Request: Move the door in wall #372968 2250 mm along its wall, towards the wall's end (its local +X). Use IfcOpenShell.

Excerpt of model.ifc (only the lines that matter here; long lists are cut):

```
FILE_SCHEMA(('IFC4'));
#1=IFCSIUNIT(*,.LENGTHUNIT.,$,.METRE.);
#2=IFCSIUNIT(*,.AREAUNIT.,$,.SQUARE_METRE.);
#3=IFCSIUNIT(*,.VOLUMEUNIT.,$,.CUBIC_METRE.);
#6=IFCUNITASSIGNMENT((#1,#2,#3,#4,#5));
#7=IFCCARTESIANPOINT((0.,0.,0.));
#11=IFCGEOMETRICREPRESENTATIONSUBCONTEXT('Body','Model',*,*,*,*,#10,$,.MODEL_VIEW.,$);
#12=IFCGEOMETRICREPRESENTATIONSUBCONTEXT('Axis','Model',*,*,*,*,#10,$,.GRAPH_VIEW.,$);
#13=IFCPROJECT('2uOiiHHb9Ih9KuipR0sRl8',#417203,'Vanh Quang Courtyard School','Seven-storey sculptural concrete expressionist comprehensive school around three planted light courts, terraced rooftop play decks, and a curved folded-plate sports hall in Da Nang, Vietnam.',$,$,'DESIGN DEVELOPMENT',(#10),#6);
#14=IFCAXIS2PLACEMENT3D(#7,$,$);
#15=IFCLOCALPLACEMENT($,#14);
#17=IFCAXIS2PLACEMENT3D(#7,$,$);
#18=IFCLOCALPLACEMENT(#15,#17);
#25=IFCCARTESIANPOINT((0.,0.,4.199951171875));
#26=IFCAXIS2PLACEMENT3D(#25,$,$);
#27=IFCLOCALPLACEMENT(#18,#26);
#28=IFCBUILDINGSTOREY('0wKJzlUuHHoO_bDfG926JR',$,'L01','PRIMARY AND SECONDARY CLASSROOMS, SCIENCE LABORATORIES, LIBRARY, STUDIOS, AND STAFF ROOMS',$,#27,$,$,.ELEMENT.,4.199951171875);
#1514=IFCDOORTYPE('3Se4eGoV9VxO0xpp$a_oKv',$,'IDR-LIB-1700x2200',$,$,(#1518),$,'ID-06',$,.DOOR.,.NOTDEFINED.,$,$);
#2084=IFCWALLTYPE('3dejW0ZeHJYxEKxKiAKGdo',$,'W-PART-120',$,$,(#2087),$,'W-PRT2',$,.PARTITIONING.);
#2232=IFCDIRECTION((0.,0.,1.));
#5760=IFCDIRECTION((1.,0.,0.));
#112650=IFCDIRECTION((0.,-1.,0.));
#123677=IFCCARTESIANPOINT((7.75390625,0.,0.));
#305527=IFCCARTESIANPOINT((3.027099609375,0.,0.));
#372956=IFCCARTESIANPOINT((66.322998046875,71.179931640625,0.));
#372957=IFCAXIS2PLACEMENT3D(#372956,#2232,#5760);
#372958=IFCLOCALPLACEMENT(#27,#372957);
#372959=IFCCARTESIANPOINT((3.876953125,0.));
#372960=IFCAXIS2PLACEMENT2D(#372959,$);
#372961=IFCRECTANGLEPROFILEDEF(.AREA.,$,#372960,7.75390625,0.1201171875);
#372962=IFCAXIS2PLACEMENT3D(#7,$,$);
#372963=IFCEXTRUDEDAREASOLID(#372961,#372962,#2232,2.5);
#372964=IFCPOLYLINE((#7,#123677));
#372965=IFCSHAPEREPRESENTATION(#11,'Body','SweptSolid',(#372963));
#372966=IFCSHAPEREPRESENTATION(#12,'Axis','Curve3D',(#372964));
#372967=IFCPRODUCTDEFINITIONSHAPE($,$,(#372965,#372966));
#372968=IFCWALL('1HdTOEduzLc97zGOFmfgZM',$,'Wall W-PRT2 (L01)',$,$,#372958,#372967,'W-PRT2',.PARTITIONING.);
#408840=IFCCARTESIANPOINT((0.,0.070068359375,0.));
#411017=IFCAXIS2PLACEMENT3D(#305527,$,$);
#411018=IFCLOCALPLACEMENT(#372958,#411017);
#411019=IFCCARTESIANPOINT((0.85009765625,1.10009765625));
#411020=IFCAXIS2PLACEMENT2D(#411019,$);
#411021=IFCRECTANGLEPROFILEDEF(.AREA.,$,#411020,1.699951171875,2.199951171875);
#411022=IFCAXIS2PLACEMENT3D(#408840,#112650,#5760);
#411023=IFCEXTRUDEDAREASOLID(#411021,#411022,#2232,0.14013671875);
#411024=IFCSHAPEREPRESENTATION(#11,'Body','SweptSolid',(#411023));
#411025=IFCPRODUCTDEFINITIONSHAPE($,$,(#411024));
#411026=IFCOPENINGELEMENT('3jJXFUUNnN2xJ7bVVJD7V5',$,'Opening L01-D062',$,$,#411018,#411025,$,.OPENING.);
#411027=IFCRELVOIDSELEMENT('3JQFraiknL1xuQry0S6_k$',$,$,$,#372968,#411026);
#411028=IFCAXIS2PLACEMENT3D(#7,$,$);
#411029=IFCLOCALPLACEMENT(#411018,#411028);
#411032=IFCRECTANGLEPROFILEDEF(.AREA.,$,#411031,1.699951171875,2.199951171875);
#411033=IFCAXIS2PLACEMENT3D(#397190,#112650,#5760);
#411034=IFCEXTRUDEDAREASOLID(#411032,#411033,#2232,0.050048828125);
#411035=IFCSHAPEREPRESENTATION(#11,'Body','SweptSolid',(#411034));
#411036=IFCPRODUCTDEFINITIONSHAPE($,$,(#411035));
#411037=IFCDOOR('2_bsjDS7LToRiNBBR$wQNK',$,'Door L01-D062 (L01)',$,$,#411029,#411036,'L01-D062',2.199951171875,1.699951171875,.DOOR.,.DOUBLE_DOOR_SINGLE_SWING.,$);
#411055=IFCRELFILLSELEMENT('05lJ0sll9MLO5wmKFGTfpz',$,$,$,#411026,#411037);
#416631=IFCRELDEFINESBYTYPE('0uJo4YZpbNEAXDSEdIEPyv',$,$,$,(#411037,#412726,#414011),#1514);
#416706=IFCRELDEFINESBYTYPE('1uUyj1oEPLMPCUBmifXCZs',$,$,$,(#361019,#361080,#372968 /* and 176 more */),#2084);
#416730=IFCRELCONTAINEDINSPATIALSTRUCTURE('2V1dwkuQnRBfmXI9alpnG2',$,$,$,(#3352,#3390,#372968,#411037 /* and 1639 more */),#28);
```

```python
import ifcopenshell
import ifcopenshell.api.geometry
import ifcopenshell.util.placement

model = ifcopenshell.open("model.ifc")

door = model.by_guid("2_bsjDS7LToRiNBBR$wQNK")
opening = door.FillsVoids[0].RelatingOpeningElement
wall = opening.VoidsElements[0].RelatingBuildingElement

wall_matrix = ifcopenshell.util.placement.get_local_placement(wall.ObjectPlacement)
shift = wall_matrix[:3, 0] * 2.25
before = ifcopenshell.util.placement.get_local_placement(door.ObjectPlacement)[:3, 3].copy()

# The door is placed relative to its opening, so it follows when the opening moves.
matrix = ifcopenshell.util.placement.get_local_placement(opening.ObjectPlacement)
matrix[:3, 3] += shift
ifcopenshell.api.geometry.edit_object_placement(
    model, product=opening, matrix=matrix, is_si=False, should_transform_children=True
)

after = ifcopenshell.util.placement.get_local_placement(door.ObjectPlacement)[:3, 3]
print("door moved by", (after - before).round(3) + 0.0)

model.write("model_rev.ifc")
```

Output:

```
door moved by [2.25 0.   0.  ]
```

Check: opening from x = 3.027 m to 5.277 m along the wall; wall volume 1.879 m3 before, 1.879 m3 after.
